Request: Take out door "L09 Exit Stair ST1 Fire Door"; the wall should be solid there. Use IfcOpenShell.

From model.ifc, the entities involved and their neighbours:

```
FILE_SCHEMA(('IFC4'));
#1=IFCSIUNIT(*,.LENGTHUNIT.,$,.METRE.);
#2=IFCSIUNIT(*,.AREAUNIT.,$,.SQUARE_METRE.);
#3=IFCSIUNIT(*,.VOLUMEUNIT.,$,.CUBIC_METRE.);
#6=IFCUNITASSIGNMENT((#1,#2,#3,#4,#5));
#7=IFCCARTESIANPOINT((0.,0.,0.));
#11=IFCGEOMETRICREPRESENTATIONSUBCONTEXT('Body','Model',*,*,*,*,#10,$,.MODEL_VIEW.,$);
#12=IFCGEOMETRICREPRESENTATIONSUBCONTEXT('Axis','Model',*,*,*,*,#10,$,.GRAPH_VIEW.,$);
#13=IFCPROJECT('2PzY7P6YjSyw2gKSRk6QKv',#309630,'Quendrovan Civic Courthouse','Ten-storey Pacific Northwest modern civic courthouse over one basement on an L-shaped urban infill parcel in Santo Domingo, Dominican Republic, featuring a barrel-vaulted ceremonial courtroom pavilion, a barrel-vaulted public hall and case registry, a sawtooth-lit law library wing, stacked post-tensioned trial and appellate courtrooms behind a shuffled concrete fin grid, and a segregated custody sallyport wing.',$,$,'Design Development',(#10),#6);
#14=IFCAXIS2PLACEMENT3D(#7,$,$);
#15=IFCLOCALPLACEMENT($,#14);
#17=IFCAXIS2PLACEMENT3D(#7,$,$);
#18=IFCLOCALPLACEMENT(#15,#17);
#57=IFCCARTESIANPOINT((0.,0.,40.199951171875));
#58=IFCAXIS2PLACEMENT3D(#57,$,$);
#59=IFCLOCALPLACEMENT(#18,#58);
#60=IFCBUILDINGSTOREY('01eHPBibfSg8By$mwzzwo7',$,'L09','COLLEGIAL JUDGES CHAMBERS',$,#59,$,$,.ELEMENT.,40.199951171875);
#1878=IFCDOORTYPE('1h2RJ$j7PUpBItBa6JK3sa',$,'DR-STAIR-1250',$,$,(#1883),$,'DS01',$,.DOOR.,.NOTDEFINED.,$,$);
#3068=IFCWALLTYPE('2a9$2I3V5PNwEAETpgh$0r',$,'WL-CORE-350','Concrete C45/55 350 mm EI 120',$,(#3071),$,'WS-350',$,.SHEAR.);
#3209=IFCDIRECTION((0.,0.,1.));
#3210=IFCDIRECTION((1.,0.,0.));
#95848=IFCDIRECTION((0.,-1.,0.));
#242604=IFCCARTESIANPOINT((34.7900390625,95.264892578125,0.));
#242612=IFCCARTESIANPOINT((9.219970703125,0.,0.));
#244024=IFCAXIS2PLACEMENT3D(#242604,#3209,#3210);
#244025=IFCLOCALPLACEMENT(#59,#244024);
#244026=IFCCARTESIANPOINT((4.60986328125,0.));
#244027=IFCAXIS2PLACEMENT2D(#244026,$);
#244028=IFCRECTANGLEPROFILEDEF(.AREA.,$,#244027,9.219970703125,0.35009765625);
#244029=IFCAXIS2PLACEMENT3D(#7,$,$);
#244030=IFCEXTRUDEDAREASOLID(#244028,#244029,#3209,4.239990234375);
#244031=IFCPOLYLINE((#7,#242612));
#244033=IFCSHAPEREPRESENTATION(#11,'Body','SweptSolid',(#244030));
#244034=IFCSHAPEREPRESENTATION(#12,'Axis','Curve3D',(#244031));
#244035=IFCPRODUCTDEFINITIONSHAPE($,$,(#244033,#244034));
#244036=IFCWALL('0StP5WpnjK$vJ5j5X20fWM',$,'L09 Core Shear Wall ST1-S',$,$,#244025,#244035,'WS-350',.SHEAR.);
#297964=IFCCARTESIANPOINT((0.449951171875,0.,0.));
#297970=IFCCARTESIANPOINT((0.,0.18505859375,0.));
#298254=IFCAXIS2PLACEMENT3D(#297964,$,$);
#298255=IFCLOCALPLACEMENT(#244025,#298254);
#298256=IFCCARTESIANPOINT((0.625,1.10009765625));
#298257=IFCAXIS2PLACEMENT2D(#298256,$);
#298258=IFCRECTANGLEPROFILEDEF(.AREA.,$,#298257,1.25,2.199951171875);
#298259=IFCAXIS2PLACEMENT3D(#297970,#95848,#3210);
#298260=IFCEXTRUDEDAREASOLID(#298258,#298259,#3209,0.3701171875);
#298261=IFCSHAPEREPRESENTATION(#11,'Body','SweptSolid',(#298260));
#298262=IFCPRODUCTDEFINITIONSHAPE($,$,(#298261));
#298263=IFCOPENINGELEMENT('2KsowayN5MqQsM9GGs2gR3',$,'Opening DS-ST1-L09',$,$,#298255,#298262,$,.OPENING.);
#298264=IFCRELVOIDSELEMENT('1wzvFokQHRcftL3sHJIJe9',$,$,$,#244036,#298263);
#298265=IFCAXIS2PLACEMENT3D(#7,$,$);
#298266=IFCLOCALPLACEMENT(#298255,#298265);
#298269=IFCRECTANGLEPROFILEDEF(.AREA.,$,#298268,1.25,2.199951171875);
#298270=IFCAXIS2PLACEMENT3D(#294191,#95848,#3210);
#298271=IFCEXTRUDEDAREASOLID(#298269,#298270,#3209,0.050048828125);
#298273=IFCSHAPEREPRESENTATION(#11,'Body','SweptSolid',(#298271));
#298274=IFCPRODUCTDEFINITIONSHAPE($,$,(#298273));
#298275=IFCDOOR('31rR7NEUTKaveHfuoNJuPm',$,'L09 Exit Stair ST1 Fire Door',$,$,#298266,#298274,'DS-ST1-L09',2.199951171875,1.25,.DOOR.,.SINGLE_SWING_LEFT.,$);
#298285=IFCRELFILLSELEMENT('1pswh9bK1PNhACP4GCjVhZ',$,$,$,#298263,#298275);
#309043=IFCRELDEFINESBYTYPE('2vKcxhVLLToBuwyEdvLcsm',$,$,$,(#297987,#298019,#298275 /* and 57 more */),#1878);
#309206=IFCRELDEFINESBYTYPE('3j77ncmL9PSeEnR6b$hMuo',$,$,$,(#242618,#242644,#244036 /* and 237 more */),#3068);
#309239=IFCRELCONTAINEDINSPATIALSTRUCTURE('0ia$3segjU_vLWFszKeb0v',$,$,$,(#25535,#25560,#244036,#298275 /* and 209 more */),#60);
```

```python
import ifcopenshell
import ifcopenshell.api.feature
import ifcopenshell.api.root
import ifcopenshell.geom
import ifcopenshell.util.shape

model = ifcopenshell.open("model.ifc")
settings = ifcopenshell.geom.settings()


def volume(element):
    """Net volume in cubic metres, openings subtracted."""
    shape = ifcopenshell.geom.create_shape(settings, element)
    return ifcopenshell.util.shape.get_volume(shape.geometry)


door = model.by_guid("31rR7NEUTKaveHfuoNJuPm")
opening = door.FillsVoids[0].RelatingOpeningElement
wall = opening.VoidsElements[0].RelatingBuildingElement
before = volume(wall)

ifcopenshell.api.root.remove_product(model, product=door)
ifcopenshell.api.feature.remove_feature(model, feature=opening)

after = volume(wall)

print(f"wall volume {before:.3f} -> {after:.3f} m3")

model.write("model_edited.ifc")
```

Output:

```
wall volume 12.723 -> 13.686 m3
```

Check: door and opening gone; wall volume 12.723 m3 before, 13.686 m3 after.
